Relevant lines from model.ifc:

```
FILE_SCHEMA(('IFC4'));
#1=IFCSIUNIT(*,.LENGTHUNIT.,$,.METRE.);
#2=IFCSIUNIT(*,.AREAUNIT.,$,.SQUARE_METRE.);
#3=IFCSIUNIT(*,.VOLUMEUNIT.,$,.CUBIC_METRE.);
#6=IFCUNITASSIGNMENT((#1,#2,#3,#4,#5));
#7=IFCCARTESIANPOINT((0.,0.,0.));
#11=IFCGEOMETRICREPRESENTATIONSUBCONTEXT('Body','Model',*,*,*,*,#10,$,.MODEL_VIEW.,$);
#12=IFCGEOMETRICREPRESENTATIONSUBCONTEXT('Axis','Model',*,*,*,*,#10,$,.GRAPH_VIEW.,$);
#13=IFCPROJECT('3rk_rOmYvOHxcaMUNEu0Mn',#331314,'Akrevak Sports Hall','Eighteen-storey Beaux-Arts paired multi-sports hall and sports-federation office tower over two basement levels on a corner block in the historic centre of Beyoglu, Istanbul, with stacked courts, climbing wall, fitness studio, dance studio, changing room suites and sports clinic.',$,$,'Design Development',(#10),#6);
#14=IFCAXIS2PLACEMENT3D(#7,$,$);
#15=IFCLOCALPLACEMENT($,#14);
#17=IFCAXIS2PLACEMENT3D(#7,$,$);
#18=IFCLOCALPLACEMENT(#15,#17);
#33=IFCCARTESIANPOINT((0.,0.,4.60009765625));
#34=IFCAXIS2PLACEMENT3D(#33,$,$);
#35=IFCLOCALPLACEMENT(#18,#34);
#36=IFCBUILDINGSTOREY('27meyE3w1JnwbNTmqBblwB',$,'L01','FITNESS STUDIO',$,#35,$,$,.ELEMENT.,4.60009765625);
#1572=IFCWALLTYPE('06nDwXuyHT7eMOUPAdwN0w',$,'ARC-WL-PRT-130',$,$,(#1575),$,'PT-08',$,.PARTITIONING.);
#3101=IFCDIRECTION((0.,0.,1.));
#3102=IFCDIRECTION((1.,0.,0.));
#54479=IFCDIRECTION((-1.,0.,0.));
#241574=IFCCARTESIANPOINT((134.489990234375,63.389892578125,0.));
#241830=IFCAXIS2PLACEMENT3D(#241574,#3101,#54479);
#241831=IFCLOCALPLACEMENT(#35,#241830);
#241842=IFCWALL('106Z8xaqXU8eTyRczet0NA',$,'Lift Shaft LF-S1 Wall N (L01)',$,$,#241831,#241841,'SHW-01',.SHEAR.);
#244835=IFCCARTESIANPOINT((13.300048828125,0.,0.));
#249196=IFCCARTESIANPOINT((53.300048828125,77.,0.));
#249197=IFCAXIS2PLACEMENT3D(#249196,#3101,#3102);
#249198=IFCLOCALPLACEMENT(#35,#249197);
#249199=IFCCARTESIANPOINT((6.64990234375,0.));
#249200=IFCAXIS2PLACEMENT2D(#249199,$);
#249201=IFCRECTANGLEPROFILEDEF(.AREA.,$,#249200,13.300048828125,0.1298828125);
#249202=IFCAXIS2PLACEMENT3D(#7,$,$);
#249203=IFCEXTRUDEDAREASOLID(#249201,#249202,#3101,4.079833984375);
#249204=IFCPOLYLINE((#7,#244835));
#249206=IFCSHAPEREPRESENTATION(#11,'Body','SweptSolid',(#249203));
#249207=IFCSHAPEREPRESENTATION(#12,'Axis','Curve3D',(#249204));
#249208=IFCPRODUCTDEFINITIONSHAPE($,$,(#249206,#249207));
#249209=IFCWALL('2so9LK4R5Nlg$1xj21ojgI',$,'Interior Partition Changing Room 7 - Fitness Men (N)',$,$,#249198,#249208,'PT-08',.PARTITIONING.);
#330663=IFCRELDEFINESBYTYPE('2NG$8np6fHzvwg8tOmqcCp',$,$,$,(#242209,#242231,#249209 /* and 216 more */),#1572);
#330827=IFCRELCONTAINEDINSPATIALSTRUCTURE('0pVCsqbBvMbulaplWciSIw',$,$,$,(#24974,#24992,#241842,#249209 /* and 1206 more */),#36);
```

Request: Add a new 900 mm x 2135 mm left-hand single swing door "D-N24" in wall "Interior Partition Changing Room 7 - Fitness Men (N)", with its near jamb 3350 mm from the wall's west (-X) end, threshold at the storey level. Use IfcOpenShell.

```python
import numpy as np
import ifcopenshell
import ifcopenshell.api.feature
import ifcopenshell.api.geometry
import ifcopenshell.api.root
import ifcopenshell.api.spatial
import ifcopenshell.geom
import ifcopenshell.util.element
import ifcopenshell.util.placement
import ifcopenshell.util.representation
import ifcopenshell.util.shape
import ifcopenshell.util.unit

model = ifcopenshell.open("model.ifc")
unit_scale = ifcopenshell.util.unit.calculate_unit_scale(model)
settings = ifcopenshell.geom.settings()


def volume(element):
    """Net volume in cubic metres, openings subtracted."""
    shape = ifcopenshell.geom.create_shape(settings, element)
    return ifcopenshell.util.shape.get_volume(shape.geometry)


wall = model.by_guid("2so9LK4R5Nlg$1xj21ojgI")
storey = ifcopenshell.util.element.get_container(wall, ifc_class="IfcBuildingStorey")
context = ifcopenshell.util.representation.get_context(model, "Model", "Body", "MODEL_VIEW")
before = volume(wall)

width, height, from_end, sill = 0.9, 2.135, 3.35, 0.0  # metres

# The wall runs along its own X axis, and the end named is its -X end.
wall_shape = ifcopenshell.geom.create_shape(settings, wall)
x, y, z = ifcopenshell.util.shape.get_vertices(wall_shape.geometry).T
start = x.min() + from_end
face, thickness = float(y.min()), float(y.max() - y.min())
wall_matrix = ifcopenshell.util.placement.get_local_placement(wall.ObjectPlacement)
level = ifcopenshell.util.placement.get_local_placement(storey.ObjectPlacement)[2, 3]


def in_wall(x, y):
    """Placement at x, y metres in the wall's axes, at sill height."""
    matrix = wall_matrix.copy()
    matrix[:, 3] = wall_matrix @ np.array([x / unit_scale, y / unit_scale, 0.0, 1.0])
    matrix[2, 3] = level + sill / unit_scale
    return matrix


# Opening: a box that overshoots both wall faces by 50 mm.
opening = ifcopenshell.api.root.create_entity(model, ifc_class="IfcOpeningElement", predefined_type="OPENING")
box = ifcopenshell.api.geometry.add_wall_representation(
    model, context=context, length=width, height=height, thickness=thickness + 0.1
)
ifcopenshell.api.geometry.assign_representation(model, product=opening, representation=box)
ifcopenshell.api.geometry.edit_object_placement(model, product=opening, matrix=in_wall(start, face - 0.05), is_si=False)
ifcopenshell.api.feature.add_feature(model, feature=opening, element=wall)

door = ifcopenshell.api.root.create_entity(model, ifc_class="IfcDoor", name="D-N24", predefined_type="DOOR")
door.OverallWidth, door.OverallHeight = width / unit_scale, height / unit_scale
door.OperationType = "SINGLE_SWING_LEFT"
body = ifcopenshell.api.geometry.add_door_representation(
    model,
    context=context,
    overall_width=door.OverallWidth,
    overall_height=door.OverallHeight,
    operation_type="SINGLE_SWING_LEFT",
    lining_properties={"LiningDepth": thickness / unit_scale, "ThresholdDepth": thickness / unit_scale},
)
ifcopenshell.api.geometry.assign_representation(model, product=door, representation=body)
ifcopenshell.api.spatial.assign_container(model, products=[door], relating_structure=storey)
ifcopenshell.api.feature.add_filling(model, opening=opening, element=door)

# The lining spans the wall, so the door starts at the wall face.
ifcopenshell.api.geometry.edit_object_placement(model, product=door, matrix=in_wall(start, face), is_si=False)

after = volume(wall)

print(f"wall volume {before:.3f} -> {after:.3f} m3")

model.write("model_updated.ifc")
```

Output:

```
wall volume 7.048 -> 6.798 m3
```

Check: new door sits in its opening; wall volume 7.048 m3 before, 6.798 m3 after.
